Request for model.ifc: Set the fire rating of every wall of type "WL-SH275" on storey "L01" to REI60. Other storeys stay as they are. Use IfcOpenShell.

First a look at what the model holds.

```python
import ifcopenshell
import ifcopenshell.util.element

model = ifcopenshell.open("model.ifc")
print(model.schema)
storey = next(s for s in model.by_type("IfcBuildingStorey") if s.Name == "L01")
walls = [e for e in ifcopenshell.util.element.get_decomposition(storey) if e.is_a("IfcWall")]
seen = {}
for e in walls:
    element_type = ifcopenshell.util.element.get_type(e)
    key = (element_type.Name if element_type != e and element_type else None, ifcopenshell.util.element.get_pset(e, "Pset_WallCommon", "FireRating"))
    seen[key] = seen.get(key, 0) + 1
for (name, value), count in sorted(seen.items(), key=str):
    print(count, "x", name, "|", value)
```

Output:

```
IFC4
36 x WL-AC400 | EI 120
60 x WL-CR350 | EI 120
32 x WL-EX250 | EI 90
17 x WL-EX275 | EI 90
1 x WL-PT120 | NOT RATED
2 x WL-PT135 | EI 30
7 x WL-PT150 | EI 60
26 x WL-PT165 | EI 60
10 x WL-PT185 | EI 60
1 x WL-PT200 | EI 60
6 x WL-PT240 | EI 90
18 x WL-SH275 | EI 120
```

```python
import ifcopenshell
import ifcopenshell.api.pset
import ifcopenshell.util.element

model = ifcopenshell.open("model.ifc")

storey = next(s for s in model.by_type("IfcBuildingStorey") if s.Name == "L01")
walls = [e for e in ifcopenshell.util.element.get_decomposition(storey) if e.is_a("IfcWall")]

count = 0
for e in walls:
    element_type = ifcopenshell.util.element.get_type(e)
    if element_type in (None, e) or element_type.Name != "WL-SH275":
        continue
    # add_pset returns the element's existing set when there is one.
    pset = ifcopenshell.api.pset.add_pset(model, product=e, name="Pset_WallCommon")
    ifcopenshell.api.pset.edit_pset(model, pset=pset, properties={"FireRating": "REI60"})
    count += 1

print(count, "walls updated")

model.write("model_rev.ifc")
```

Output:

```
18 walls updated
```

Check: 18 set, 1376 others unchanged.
